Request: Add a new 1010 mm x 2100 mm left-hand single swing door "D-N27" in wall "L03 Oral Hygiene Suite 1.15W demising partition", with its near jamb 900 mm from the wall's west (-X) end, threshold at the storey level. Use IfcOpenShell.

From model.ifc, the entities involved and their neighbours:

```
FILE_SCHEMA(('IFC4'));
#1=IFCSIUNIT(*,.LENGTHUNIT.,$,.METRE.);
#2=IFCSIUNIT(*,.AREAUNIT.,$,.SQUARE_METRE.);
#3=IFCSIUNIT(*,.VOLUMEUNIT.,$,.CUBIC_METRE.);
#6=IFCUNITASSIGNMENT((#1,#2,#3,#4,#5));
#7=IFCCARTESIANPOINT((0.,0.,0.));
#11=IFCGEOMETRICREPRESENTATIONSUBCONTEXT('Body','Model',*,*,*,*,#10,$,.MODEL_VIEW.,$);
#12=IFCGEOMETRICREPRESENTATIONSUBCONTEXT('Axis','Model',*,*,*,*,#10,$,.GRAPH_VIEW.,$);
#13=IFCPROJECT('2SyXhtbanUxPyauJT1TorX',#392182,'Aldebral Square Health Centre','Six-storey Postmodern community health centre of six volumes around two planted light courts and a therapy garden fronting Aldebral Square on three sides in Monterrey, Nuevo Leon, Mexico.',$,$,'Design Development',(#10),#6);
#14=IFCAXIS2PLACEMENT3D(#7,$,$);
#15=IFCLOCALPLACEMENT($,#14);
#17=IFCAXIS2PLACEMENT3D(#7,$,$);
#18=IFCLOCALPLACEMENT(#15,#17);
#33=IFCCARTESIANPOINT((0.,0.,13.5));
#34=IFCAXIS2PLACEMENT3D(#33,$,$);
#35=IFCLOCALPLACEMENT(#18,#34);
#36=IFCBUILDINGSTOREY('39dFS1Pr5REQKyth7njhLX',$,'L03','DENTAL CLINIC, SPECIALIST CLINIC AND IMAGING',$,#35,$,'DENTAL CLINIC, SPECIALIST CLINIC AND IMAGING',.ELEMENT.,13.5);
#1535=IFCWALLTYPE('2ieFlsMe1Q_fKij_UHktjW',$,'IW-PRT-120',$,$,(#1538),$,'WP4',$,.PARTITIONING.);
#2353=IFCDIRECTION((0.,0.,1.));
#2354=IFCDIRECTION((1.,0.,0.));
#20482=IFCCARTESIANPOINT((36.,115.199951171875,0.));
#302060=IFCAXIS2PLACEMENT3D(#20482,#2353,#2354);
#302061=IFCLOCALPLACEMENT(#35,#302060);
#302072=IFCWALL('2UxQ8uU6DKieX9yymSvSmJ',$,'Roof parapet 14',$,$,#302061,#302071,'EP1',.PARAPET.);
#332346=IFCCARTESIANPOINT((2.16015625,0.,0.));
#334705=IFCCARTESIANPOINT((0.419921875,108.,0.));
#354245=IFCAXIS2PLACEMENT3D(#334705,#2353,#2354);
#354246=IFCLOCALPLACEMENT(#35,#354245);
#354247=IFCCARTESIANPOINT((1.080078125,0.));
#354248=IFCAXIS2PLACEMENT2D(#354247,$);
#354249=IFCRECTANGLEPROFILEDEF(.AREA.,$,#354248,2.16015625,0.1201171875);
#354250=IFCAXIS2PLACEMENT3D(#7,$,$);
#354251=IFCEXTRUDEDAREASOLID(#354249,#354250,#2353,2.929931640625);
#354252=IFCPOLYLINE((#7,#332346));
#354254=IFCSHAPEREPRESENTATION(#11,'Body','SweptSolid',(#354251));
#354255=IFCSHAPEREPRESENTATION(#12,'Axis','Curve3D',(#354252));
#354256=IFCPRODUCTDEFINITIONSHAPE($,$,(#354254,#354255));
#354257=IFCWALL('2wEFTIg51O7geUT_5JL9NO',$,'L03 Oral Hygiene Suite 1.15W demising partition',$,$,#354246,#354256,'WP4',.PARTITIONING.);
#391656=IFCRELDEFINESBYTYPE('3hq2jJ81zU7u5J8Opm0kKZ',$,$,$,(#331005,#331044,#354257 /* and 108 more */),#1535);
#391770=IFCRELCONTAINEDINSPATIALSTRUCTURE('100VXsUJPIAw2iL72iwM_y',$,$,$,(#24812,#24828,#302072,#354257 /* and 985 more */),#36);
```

```python
import numpy as np
import ifcopenshell
import ifcopenshell.api.feature
import ifcopenshell.api.geometry
import ifcopenshell.api.root
import ifcopenshell.api.spatial
import ifcopenshell.geom
import ifcopenshell.util.element
import ifcopenshell.util.placement
import ifcopenshell.util.representation
import ifcopenshell.util.shape
import ifcopenshell.util.unit

model = ifcopenshell.open("model.ifc")
unit_scale = ifcopenshell.util.unit.calculate_unit_scale(model)
settings = ifcopenshell.geom.settings()


def volume(element):
    """Net volume in cubic metres, openings subtracted."""
    shape = ifcopenshell.geom.create_shape(settings, element)
    return ifcopenshell.util.shape.get_volume(shape.geometry)


wall = model.by_id(354257)
storey = ifcopenshell.util.element.get_container(wall, ifc_class="IfcBuildingStorey")
context = ifcopenshell.util.representation.get_context(model, "Model", "Body", "MODEL_VIEW")
before = volume(wall)

width, height, from_end, sill = 1.01, 2.1, 0.9, 0.0  # metres

# The wall runs along its own X axis, and the end named is its -X end.
wall_shape = ifcopenshell.geom.create_shape(settings, wall)
x, y, z = ifcopenshell.util.shape.get_vertices(wall_shape.geometry).T
start = x.min() + from_end
face, thickness = float(y.min()), float(y.max() - y.min())
wall_matrix = ifcopenshell.util.placement.get_local_placement(wall.ObjectPlacement)
level = ifcopenshell.util.placement.get_local_placement(storey.ObjectPlacement)[2, 3]


def in_wall(x, y):
    """Placement at x, y metres in the wall's axes, at sill height."""
    matrix = wall_matrix.copy()
    matrix[:, 3] = wall_matrix @ np.array([x / unit_scale, y / unit_scale, 0.0, 1.0])
    matrix[2, 3] = level + sill / unit_scale
    return matrix


# Opening: a box that overshoots both wall faces by 50 mm.
opening = ifcopenshell.api.root.create_entity(model, ifc_class="IfcOpeningElement", predefined_type="OPENING")
box = ifcopenshell.api.geometry.add_wall_representation(
    model, context=context, length=width, height=height, thickness=thickness + 0.1
)
ifcopenshell.api.geometry.assign_representation(model, product=opening, representation=box)
ifcopenshell.api.geometry.edit_object_placement(model, product=opening, matrix=in_wall(start, face - 0.05), is_si=False)
ifcopenshell.api.feature.add_feature(model, feature=opening, element=wall)

door = ifcopenshell.api.root.create_entity(model, ifc_class="IfcDoor", name="D-N27", predefined_type="DOOR")
door.OverallWidth, door.OverallHeight = width / unit_scale, height / unit_scale
door.OperationType = "SINGLE_SWING_LEFT"
body = ifcopenshell.api.geometry.add_door_representation(
    model,
    context=context,
    overall_width=door.OverallWidth,
    overall_height=door.OverallHeight,
    operation_type="SINGLE_SWING_LEFT",
    lining_properties={"LiningDepth": thickness / unit_scale, "ThresholdDepth": thickness / unit_scale},
)
ifcopenshell.api.geometry.assign_representation(model, product=door, representation=body)
ifcopenshell.api.spatial.assign_container(model, products=[door], relating_structure=storey)
ifcopenshell.api.feature.add_filling(model, opening=opening, element=door)

# The lining spans the wall, so the door starts at the wall face.
ifcopenshell.api.geometry.edit_object_placement(model, product=door, matrix=in_wall(start, face), is_si=False)

after = volume(wall)

print(f"wall volume {before:.3f} -> {after:.3f} m3")

model.write("model_updated.ifc")
```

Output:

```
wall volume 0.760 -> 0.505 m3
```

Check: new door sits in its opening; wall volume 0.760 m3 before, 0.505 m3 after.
